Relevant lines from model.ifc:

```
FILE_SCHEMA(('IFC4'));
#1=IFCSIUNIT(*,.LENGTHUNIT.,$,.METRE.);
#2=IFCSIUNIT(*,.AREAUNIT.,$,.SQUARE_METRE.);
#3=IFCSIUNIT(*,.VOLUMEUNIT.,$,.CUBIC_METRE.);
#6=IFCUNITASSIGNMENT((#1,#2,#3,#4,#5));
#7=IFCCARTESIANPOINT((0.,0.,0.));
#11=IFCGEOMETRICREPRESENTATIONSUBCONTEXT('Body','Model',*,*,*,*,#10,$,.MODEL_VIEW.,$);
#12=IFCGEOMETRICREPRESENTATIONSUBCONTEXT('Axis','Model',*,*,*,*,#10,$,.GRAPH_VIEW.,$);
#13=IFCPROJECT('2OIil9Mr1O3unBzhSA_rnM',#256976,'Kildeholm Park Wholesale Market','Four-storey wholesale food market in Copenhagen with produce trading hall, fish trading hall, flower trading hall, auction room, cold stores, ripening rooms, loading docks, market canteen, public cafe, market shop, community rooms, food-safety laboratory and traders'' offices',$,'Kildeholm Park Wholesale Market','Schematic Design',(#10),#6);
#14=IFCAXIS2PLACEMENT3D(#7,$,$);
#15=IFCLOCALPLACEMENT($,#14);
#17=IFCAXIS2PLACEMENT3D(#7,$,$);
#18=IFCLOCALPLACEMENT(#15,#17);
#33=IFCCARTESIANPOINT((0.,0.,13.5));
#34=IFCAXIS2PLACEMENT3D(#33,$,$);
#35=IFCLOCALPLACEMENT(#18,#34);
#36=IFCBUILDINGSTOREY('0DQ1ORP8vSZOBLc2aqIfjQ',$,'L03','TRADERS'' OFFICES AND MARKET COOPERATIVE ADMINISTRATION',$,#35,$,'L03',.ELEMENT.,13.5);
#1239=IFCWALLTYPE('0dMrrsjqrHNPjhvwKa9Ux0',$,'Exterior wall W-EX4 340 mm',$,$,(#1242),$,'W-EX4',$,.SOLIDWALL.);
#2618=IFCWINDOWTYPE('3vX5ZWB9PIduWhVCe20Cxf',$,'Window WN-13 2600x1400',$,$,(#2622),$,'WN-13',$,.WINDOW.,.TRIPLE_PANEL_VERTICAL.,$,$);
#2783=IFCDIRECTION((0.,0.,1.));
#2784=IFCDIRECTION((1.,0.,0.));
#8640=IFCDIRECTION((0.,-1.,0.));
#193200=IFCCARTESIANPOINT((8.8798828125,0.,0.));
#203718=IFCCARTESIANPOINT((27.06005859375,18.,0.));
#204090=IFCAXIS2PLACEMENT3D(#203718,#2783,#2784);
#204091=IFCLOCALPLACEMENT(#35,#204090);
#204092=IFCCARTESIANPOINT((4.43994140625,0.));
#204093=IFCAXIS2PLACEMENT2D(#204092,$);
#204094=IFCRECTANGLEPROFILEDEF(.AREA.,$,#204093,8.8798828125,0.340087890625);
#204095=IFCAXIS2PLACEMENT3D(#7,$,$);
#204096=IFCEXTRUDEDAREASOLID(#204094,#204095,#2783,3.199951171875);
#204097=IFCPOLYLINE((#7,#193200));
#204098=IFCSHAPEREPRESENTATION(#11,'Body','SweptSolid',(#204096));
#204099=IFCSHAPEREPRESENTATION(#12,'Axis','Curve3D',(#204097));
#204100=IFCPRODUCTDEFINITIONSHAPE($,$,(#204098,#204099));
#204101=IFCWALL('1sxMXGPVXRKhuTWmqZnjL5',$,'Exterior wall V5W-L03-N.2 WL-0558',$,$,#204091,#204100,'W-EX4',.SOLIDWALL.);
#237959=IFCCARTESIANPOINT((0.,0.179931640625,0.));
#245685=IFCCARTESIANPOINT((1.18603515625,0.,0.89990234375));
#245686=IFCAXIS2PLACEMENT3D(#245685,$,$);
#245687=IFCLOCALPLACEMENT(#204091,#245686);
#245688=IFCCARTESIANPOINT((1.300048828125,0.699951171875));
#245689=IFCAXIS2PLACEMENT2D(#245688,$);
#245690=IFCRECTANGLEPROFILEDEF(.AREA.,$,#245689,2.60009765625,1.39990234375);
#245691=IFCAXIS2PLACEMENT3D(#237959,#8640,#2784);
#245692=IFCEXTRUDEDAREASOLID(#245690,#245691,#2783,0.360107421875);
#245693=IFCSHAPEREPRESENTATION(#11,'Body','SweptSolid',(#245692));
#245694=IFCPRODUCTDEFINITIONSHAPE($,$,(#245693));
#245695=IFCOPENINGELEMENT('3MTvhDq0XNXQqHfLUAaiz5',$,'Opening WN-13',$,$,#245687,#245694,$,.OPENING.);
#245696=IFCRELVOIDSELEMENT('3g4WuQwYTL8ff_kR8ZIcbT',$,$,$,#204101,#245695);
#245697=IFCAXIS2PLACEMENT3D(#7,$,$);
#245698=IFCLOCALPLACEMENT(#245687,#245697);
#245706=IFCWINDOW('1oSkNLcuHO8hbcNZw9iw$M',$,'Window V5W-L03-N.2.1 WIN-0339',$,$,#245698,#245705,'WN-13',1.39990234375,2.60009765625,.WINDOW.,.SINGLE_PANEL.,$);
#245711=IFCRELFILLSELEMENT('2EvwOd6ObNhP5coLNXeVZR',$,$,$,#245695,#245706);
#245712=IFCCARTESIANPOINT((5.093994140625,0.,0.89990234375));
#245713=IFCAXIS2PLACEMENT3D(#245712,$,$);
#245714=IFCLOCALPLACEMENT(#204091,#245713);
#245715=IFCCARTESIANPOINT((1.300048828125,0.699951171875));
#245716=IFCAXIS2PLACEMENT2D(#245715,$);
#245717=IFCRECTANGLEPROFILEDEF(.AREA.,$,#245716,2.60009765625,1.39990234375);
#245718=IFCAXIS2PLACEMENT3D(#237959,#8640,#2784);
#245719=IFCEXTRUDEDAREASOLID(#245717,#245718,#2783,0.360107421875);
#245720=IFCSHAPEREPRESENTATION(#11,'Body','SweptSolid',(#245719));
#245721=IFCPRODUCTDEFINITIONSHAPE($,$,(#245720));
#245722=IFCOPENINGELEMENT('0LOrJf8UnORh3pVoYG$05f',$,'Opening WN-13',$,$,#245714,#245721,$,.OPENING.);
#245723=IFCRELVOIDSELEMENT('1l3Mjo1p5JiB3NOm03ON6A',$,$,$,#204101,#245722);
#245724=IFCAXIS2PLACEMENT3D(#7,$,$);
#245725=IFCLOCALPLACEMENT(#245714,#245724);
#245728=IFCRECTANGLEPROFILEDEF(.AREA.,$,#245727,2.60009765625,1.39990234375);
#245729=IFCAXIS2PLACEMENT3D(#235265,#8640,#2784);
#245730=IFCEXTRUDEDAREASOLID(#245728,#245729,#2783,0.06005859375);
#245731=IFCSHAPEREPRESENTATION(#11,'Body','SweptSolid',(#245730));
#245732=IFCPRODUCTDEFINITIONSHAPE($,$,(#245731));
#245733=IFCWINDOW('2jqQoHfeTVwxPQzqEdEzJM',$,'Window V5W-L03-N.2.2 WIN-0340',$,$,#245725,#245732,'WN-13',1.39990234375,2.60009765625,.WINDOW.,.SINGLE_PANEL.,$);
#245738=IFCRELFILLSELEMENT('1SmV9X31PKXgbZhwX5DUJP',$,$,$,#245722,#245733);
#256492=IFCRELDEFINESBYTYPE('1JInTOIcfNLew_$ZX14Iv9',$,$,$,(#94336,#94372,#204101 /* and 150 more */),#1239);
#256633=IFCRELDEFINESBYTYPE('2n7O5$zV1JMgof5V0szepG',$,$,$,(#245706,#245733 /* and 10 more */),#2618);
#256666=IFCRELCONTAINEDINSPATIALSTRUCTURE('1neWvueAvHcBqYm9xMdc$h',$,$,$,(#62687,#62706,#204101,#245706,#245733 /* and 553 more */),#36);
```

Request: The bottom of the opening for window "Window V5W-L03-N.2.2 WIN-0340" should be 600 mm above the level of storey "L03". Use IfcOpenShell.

```python
import numpy as np
import ifcopenshell
import ifcopenshell.api.geometry
import ifcopenshell.geom
import ifcopenshell.util.element
import ifcopenshell.util.placement
import ifcopenshell.util.shape
import ifcopenshell.util.unit

model = ifcopenshell.open("model.ifc")
unit_scale = ifcopenshell.util.unit.calculate_unit_scale(model)

window = model.by_id(245733)
opening = window.FillsVoids[0].RelatingOpeningElement
storey = ifcopenshell.util.element.get_container(window, ifc_class="IfcBuildingStorey")
level = ifcopenshell.util.placement.get_local_placement(storey.ObjectPlacement)[2, 3]

# The opening's origin need not be at the sill, so measure its lowest point.
shape = ifcopenshell.geom.create_shape(ifcopenshell.geom.settings(), opening)
bottom = ifcopenshell.util.shape.get_shape_bottom_elevation(shape, shape.geometry) / unit_scale
dz = level + 0.6 - bottom

shift = np.array([0.0, 0.0, dz])
# The window is placed relative to its opening, so it follows when the opening moves.
matrix = ifcopenshell.util.placement.get_local_placement(opening.ObjectPlacement)
matrix[:3, 3] += shift
ifcopenshell.api.geometry.edit_object_placement(
    model, product=opening, matrix=matrix, is_si=False, should_transform_children=True
)

print(f"moved by {dz * unit_scale:+.3f} m")

model.write("model_updated.ifc")
```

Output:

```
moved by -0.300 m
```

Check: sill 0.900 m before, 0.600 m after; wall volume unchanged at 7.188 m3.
